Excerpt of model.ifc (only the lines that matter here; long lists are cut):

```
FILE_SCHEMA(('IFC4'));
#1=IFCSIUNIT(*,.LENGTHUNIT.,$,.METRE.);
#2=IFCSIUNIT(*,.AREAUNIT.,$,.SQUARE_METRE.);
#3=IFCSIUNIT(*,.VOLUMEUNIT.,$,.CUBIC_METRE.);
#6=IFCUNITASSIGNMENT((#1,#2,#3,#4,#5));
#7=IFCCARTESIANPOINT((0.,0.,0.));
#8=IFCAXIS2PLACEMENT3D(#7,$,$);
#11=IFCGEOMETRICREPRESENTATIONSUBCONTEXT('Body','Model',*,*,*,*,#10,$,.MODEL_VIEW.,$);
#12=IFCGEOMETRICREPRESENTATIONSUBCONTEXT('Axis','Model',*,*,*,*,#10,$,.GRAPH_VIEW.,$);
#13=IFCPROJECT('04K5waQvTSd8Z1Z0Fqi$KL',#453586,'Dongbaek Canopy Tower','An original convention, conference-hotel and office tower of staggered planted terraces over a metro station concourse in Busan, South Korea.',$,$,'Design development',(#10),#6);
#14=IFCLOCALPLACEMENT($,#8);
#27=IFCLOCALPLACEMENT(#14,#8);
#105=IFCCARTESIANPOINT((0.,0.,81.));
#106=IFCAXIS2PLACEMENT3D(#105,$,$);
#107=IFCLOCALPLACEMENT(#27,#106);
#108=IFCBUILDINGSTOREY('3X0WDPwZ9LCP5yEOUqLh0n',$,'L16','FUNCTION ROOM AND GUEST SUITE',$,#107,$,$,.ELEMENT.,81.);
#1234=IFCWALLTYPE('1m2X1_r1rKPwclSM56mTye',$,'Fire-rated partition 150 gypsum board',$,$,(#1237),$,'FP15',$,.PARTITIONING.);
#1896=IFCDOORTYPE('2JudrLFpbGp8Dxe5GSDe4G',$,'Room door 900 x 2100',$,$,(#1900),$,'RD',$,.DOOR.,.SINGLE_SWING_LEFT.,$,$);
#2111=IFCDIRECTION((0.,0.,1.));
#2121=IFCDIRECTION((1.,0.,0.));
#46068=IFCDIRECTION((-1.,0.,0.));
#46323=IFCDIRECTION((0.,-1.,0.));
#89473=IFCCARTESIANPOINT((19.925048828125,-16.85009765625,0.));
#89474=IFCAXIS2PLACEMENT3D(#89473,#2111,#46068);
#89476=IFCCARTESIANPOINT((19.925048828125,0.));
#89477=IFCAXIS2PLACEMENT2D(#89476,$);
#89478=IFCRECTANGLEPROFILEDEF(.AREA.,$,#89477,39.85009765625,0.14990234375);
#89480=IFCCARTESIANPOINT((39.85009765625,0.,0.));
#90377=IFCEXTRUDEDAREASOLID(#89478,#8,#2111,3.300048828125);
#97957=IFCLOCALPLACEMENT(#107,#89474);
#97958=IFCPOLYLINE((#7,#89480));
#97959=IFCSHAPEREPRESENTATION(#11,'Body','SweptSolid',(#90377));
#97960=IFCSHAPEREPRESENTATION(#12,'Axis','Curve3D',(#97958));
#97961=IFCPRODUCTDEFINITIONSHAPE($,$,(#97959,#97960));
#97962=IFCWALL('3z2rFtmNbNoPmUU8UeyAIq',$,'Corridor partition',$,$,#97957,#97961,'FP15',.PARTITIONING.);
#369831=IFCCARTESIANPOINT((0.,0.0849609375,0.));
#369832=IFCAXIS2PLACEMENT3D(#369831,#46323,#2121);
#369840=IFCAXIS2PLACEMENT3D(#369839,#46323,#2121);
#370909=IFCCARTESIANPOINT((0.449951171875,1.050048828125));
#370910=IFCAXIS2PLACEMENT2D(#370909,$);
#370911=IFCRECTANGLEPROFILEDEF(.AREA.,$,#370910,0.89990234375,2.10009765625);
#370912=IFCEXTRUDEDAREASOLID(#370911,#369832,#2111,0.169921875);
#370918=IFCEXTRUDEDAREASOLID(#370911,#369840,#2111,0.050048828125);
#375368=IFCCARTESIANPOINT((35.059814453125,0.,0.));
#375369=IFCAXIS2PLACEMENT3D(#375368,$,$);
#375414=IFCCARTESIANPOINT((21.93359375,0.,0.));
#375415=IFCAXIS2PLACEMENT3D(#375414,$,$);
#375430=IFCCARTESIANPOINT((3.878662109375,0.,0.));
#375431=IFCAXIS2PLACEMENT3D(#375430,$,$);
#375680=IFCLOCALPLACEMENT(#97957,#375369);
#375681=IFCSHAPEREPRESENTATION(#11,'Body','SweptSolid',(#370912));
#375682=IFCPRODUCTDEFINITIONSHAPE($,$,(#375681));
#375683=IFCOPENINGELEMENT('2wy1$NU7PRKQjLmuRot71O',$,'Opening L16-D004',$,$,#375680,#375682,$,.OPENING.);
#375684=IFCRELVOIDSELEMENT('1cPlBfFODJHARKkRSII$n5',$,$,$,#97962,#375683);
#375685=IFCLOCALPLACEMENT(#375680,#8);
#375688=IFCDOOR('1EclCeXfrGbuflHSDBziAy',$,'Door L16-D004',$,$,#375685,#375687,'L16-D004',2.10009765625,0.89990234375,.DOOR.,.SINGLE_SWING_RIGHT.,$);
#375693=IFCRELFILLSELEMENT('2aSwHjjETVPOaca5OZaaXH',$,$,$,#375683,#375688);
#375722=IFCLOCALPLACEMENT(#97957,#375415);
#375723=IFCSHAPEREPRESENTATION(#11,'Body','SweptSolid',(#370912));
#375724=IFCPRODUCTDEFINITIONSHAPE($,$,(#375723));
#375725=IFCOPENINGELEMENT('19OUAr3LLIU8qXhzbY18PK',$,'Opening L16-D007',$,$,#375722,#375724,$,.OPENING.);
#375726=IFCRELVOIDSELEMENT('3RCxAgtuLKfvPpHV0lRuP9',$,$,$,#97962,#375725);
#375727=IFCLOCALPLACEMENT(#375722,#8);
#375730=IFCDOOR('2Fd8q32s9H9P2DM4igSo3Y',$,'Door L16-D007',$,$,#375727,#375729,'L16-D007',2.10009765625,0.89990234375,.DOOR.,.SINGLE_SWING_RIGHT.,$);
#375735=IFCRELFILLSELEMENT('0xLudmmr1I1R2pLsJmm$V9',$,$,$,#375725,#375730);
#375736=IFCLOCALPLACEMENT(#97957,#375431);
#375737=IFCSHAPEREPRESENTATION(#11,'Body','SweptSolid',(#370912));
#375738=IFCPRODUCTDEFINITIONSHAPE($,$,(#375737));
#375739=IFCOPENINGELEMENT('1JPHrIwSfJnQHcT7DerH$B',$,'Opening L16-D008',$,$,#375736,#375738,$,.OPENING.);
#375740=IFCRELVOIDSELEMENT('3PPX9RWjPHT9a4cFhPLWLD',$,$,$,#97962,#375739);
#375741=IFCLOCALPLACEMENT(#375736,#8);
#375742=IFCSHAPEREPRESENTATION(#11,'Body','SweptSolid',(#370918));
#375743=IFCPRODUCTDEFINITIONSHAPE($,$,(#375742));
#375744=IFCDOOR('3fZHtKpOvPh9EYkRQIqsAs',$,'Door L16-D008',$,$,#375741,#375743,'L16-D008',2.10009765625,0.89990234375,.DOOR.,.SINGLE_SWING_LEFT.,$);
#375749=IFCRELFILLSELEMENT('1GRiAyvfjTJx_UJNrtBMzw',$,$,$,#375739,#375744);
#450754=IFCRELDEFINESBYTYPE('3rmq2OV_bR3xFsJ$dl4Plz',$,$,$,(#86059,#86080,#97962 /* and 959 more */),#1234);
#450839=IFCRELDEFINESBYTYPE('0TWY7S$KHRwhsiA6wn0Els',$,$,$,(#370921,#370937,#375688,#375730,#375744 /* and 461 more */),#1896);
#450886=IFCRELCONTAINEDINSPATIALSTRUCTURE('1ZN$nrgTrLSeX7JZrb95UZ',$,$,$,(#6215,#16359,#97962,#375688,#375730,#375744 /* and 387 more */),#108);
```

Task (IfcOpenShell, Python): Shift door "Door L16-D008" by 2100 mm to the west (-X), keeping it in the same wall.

```python
import ifcopenshell
import ifcopenshell.api.geometry
import ifcopenshell.util.placement

model = ifcopenshell.open("model.ifc")

door = model.by_guid("3fZHtKpOvPh9EYkRQIqsAs")
opening = door.FillsVoids[0].RelatingOpeningElement
wall = opening.VoidsElements[0].RelatingBuildingElement

wall_matrix = ifcopenshell.util.placement.get_local_placement(wall.ObjectPlacement)
shift = wall_matrix[:3, 0] * 2.1
before = ifcopenshell.util.placement.get_local_placement(door.ObjectPlacement)[:3, 3].copy()

# The door is placed relative to its opening, so it follows when the opening moves.
matrix = ifcopenshell.util.placement.get_local_placement(opening.ObjectPlacement)
matrix[:3, 3] += shift
ifcopenshell.api.geometry.edit_object_placement(
    model, product=opening, matrix=matrix, is_si=False, should_transform_children=True
)

after = ifcopenshell.util.placement.get_local_placement(door.ObjectPlacement)[:3, 3]
print("door moved by", (after - before).round(3) + 0.0)

model.write("model_updated.ifc")
```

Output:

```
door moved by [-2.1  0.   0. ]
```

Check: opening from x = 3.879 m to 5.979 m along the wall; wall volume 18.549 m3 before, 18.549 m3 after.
